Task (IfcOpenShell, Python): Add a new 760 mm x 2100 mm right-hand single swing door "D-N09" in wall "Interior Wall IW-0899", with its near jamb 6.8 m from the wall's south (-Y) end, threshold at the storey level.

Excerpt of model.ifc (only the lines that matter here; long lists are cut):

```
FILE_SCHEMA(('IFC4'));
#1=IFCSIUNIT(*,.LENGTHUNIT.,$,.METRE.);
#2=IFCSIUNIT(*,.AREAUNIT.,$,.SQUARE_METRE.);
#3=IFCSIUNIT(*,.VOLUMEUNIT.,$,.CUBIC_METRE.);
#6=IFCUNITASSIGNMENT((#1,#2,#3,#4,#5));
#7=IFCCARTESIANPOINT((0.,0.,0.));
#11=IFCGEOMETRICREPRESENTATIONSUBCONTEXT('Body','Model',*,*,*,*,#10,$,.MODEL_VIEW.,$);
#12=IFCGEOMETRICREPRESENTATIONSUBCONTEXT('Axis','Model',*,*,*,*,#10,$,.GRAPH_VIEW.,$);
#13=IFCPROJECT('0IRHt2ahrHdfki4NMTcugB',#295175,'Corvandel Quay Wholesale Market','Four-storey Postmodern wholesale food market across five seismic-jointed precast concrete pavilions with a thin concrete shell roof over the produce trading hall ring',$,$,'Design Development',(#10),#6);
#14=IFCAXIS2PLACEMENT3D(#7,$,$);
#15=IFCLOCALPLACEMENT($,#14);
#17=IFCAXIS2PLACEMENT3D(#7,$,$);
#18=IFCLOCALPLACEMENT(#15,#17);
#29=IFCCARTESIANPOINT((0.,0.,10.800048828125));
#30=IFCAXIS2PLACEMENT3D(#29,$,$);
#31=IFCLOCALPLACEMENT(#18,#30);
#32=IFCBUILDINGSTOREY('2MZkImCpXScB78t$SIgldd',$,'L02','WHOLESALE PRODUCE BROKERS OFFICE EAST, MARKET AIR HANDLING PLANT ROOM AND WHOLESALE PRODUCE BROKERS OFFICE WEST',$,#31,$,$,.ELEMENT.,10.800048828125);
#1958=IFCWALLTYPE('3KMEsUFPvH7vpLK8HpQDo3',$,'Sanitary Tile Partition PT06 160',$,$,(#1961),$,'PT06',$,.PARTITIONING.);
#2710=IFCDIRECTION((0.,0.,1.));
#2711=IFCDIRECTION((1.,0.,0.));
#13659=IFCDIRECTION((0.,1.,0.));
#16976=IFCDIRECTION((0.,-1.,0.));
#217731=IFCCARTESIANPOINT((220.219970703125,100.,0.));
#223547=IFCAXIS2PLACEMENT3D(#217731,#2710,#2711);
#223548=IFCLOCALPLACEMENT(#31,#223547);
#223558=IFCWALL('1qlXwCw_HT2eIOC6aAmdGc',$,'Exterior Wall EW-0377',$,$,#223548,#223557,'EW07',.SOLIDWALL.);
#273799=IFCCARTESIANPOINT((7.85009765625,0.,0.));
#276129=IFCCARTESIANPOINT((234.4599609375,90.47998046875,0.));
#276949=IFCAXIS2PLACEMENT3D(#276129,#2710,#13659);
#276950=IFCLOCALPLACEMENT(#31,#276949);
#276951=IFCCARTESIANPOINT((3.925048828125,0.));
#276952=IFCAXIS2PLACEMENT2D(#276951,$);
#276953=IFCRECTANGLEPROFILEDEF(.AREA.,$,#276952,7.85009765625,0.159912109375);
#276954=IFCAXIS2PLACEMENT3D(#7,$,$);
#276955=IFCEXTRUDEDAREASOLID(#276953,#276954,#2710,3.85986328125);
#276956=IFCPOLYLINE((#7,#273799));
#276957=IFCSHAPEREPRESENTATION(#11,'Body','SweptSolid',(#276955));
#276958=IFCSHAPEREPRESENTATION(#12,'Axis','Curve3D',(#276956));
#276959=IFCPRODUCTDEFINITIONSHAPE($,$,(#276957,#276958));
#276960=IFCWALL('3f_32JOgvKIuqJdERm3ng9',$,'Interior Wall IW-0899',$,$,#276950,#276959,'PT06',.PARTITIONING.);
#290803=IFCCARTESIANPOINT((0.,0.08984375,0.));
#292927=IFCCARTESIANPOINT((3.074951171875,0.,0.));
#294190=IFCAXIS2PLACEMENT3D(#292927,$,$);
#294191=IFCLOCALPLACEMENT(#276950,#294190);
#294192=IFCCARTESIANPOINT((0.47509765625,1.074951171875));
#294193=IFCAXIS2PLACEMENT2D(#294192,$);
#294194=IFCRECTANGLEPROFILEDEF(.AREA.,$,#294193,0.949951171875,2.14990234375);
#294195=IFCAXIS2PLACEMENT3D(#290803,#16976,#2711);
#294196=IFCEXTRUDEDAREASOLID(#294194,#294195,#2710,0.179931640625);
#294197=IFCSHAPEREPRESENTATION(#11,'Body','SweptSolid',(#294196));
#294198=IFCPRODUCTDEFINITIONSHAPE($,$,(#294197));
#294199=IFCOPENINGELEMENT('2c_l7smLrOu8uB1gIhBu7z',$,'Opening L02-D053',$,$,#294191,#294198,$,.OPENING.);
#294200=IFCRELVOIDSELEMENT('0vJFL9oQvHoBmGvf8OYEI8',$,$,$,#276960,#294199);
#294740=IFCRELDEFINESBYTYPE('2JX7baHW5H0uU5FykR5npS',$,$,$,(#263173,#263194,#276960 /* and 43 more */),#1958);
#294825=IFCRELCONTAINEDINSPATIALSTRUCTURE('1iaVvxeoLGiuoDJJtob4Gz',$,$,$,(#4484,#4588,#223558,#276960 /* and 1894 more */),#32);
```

```python
import numpy as np
import ifcopenshell
import ifcopenshell.api.feature
import ifcopenshell.api.geometry
import ifcopenshell.api.root
import ifcopenshell.api.spatial
import ifcopenshell.geom
import ifcopenshell.util.element
import ifcopenshell.util.placement
import ifcopenshell.util.representation
import ifcopenshell.util.shape
import ifcopenshell.util.unit

model = ifcopenshell.open("model.ifc")
unit_scale = ifcopenshell.util.unit.calculate_unit_scale(model)
settings = ifcopenshell.geom.settings()


def volume(element):
    """Net volume in cubic metres, openings subtracted."""
    shape = ifcopenshell.geom.create_shape(settings, element)
    return ifcopenshell.util.shape.get_volume(shape.geometry)


wall = model.by_guid("3f_32JOgvKIuqJdERm3ng9")
storey = ifcopenshell.util.element.get_container(wall, ifc_class="IfcBuildingStorey")
context = ifcopenshell.util.representation.get_context(model, "Model", "Body", "MODEL_VIEW")
before = volume(wall)

width, height, from_end, sill = 0.76, 2.1, 6.8, 0.0  # metres

# The wall runs along its own X axis, and the end named is its -X end.
wall_shape = ifcopenshell.geom.create_shape(settings, wall)
x, y, z = ifcopenshell.util.shape.get_vertices(wall_shape.geometry).T
start = x.min() + from_end
face, thickness = float(y.min()), float(y.max() - y.min())
wall_matrix = ifcopenshell.util.placement.get_local_placement(wall.ObjectPlacement)
level = ifcopenshell.util.placement.get_local_placement(storey.ObjectPlacement)[2, 3]


def in_wall(x, y):
    """Placement at x, y metres in the wall's axes, at sill height."""
    matrix = wall_matrix.copy()
    matrix[:, 3] = wall_matrix @ np.array([x / unit_scale, y / unit_scale, 0.0, 1.0])
    matrix[2, 3] = level + sill / unit_scale
    return matrix


# Opening: a box that overshoots both wall faces by 50 mm.
opening = ifcopenshell.api.root.create_entity(model, ifc_class="IfcOpeningElement", predefined_type="OPENING")
box = ifcopenshell.api.geometry.add_wall_representation(
    model, context=context, length=width, height=height, thickness=thickness + 0.1
)
ifcopenshell.api.geometry.assign_representation(model, product=opening, representation=box)
ifcopenshell.api.geometry.edit_object_placement(model, product=opening, matrix=in_wall(start, face - 0.05), is_si=False)
ifcopenshell.api.feature.add_feature(model, feature=opening, element=wall)

door = ifcopenshell.api.root.create_entity(model, ifc_class="IfcDoor", name="D-N09", predefined_type="DOOR")
door.OverallWidth, door.OverallHeight = width / unit_scale, height / unit_scale
door.OperationType = "SINGLE_SWING_RIGHT"
body = ifcopenshell.api.geometry.add_door_representation(
    model,
    context=context,
    overall_width=door.OverallWidth,
    overall_height=door.OverallHeight,
    operation_type="SINGLE_SWING_RIGHT",
    lining_properties={"LiningDepth": thickness / unit_scale, "ThresholdDepth": thickness / unit_scale},
)
ifcopenshell.api.geometry.assign_representation(model, product=door, representation=body)
ifcopenshell.api.spatial.assign_container(model, products=[door], relating_structure=storey)
ifcopenshell.api.feature.add_filling(model, opening=opening, element=door)

# The lining spans the wall, so the door starts at the wall face.
ifcopenshell.api.geometry.edit_object_placement(model, product=door, matrix=in_wall(start, face), is_si=False)

after = volume(wall)

print(f"wall volume {before:.3f} -> {after:.3f} m3")

model.write("model_v2.ifc")
```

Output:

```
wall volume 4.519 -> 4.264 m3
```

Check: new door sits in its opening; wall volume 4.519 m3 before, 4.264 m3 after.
